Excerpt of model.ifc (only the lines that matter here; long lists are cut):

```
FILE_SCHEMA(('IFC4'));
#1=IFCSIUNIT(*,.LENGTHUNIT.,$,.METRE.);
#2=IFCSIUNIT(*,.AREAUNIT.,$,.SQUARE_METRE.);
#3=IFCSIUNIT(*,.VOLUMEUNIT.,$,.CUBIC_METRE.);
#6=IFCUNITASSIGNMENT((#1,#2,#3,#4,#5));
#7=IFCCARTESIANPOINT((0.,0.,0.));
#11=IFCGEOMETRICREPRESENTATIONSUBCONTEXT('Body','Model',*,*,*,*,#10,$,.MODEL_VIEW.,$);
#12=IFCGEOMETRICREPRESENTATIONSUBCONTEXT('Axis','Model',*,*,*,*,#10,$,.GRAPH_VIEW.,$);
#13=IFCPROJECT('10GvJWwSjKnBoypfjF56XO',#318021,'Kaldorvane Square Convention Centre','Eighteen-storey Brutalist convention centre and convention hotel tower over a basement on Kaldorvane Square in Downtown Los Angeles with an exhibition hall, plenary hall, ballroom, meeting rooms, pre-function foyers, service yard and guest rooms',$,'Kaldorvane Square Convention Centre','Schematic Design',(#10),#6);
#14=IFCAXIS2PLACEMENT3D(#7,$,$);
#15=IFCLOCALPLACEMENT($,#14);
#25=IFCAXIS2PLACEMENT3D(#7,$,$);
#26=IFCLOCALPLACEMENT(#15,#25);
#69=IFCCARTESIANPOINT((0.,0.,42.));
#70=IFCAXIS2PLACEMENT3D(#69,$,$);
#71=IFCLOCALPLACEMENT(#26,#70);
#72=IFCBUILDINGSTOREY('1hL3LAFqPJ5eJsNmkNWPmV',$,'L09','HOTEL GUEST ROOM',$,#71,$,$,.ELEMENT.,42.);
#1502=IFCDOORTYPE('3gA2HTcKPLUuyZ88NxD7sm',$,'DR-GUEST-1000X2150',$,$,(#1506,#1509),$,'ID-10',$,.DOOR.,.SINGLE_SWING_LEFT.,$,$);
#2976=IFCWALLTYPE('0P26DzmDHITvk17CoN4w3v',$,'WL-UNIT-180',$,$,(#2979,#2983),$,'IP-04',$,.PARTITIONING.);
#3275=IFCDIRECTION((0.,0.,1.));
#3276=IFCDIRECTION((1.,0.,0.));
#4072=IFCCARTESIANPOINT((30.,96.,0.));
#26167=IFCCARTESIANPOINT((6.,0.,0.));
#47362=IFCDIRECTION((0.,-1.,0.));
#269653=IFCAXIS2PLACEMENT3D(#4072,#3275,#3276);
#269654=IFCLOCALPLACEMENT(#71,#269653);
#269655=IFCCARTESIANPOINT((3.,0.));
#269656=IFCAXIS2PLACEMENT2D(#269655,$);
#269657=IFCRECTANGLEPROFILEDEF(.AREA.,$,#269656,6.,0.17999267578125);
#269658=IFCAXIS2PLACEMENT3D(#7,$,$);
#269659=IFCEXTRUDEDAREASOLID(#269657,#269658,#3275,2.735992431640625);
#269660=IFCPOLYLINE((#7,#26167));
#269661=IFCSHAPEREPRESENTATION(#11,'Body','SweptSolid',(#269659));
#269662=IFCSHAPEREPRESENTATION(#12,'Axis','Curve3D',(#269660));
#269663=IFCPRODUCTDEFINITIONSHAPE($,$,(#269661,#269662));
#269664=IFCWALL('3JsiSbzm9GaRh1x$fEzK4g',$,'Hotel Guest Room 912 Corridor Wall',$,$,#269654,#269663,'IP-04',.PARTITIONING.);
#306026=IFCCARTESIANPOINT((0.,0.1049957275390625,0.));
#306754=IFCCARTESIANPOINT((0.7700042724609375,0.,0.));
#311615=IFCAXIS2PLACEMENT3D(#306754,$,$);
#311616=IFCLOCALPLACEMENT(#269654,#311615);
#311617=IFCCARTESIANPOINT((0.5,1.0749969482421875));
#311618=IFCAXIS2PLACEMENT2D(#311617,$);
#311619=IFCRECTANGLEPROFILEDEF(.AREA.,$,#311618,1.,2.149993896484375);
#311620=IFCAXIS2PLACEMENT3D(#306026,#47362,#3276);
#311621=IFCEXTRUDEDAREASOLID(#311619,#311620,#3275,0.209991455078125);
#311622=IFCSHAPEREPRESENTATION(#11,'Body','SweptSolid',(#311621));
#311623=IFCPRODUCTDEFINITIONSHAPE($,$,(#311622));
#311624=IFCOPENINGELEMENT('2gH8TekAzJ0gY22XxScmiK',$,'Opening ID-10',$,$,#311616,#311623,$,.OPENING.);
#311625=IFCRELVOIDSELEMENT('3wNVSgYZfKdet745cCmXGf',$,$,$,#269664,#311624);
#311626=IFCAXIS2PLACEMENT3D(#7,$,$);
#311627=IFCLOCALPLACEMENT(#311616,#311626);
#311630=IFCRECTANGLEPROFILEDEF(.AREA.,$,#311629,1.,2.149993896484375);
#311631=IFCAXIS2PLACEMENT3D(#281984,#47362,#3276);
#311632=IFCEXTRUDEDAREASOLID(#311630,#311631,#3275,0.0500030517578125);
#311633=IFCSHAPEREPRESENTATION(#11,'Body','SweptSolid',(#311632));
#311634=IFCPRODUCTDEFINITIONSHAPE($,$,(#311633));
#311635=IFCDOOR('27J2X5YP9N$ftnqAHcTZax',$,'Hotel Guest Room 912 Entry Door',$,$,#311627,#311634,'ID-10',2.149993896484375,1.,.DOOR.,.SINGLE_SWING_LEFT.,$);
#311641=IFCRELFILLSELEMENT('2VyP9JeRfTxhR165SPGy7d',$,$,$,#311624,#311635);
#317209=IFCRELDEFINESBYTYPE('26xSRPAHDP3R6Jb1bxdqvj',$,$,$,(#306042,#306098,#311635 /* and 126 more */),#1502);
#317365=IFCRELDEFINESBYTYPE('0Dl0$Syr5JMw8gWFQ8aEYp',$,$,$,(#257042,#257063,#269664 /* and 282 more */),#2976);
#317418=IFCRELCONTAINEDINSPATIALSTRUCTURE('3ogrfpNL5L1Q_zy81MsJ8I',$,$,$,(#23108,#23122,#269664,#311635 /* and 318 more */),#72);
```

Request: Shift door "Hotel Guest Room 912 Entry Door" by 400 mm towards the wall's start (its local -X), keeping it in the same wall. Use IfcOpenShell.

```python
import ifcopenshell
import ifcopenshell.api.geometry
import ifcopenshell.util.placement

model = ifcopenshell.open("model.ifc")

door = model.by_guid("27J2X5YP9N$ftnqAHcTZax")
opening = door.FillsVoids[0].RelatingOpeningElement
wall = opening.VoidsElements[0].RelatingBuildingElement

wall_matrix = ifcopenshell.util.placement.get_local_placement(wall.ObjectPlacement)
shift = wall_matrix[:3, 0] * -0.4
before = ifcopenshell.util.placement.get_local_placement(door.ObjectPlacement)[:3, 3].copy()

# The door is placed relative to its opening, so it follows when the opening moves.
matrix = ifcopenshell.util.placement.get_local_placement(opening.ObjectPlacement)
matrix[:3, 3] += shift
ifcopenshell.api.geometry.edit_object_placement(
    model, product=opening, matrix=matrix, is_si=False, should_transform_children=True
)

after = ifcopenshell.util.placement.get_local_placement(door.ObjectPlacement)[:3, 3]
print("door moved by", (after - before).round(3) + 0.0)

model.write("model_edited.ifc")
```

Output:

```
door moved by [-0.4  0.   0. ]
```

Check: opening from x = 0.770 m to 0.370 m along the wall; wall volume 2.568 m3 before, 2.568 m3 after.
